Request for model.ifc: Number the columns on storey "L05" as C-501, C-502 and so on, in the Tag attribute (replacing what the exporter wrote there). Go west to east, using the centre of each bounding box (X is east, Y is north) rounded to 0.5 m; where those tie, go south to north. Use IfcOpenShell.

First a look at what the model holds.

```python
import ifcopenshell
import ifcopenshell.util.element
import ifcopenshell.util.placement

model = ifcopenshell.open("model.ifc")
print(model.schema)
storey = next(s for s in model.by_type("IfcBuildingStorey") if s.Name == "L05")
columns = [e for e in ifcopenshell.util.element.get_decomposition(storey) if e.is_a("IfcColumn")]
for e in sorted(columns, key=lambda e: e.id()):
    origin = ifcopenshell.util.placement.get_local_placement(e.ObjectPlacement)[:3, 3]
    print(e.id(), e.Tag, e.Name, origin.round(2) + 0.0, sep=" | ")
```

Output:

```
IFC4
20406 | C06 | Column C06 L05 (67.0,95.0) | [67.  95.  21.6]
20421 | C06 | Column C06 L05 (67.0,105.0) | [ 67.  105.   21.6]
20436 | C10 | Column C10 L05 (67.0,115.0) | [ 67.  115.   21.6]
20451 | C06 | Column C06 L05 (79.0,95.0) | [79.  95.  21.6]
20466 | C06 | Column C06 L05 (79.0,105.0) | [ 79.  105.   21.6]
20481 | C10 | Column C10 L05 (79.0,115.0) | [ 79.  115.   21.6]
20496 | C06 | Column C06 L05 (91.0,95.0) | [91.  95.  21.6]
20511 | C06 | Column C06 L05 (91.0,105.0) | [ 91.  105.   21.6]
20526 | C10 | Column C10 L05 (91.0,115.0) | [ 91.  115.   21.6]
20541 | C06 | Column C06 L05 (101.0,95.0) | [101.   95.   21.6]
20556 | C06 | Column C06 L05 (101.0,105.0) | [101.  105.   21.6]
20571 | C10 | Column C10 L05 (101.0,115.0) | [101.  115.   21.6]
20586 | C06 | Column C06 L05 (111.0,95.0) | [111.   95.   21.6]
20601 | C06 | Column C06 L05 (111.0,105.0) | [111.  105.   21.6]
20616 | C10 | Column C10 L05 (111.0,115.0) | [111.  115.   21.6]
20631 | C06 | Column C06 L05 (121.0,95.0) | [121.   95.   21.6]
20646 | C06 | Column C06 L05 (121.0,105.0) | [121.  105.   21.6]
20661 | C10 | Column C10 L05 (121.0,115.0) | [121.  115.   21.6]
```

```python
import ifcopenshell
import ifcopenshell.geom
import ifcopenshell.util.element
import ifcopenshell.util.shape

model = ifcopenshell.open("model.ifc")
settings = ifcopenshell.geom.settings()
settings.set("use-world-coords", True)


def centre(element):
    shape = ifcopenshell.geom.create_shape(settings, element)
    return ifcopenshell.util.shape.get_bbox_centroid(shape.geometry)


storey = next(s for s in model.by_type("IfcBuildingStorey") if s.Name == "L05")
columns = [e for e in ifcopenshell.util.element.get_decomposition(storey) if e.is_a("IfcColumn")]

# Insertion points can sit at a corner or the storey origin, so sort by the geometry (in metres).
centres = {e: centre(e) for e in columns}
columns.sort(key=lambda e: (round(centres[e][0] / 0.5), centres[e][1]))

for i, e in enumerate(columns, start=1):
    number = f"C-5{i:02d}"
    e.Tag = number
    print(e.id(), number)

model.write("model-out.ifc")
```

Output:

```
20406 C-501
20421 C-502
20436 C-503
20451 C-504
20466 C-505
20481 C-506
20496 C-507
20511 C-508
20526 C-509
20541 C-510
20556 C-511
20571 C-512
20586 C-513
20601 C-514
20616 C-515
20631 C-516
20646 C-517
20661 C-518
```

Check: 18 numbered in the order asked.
